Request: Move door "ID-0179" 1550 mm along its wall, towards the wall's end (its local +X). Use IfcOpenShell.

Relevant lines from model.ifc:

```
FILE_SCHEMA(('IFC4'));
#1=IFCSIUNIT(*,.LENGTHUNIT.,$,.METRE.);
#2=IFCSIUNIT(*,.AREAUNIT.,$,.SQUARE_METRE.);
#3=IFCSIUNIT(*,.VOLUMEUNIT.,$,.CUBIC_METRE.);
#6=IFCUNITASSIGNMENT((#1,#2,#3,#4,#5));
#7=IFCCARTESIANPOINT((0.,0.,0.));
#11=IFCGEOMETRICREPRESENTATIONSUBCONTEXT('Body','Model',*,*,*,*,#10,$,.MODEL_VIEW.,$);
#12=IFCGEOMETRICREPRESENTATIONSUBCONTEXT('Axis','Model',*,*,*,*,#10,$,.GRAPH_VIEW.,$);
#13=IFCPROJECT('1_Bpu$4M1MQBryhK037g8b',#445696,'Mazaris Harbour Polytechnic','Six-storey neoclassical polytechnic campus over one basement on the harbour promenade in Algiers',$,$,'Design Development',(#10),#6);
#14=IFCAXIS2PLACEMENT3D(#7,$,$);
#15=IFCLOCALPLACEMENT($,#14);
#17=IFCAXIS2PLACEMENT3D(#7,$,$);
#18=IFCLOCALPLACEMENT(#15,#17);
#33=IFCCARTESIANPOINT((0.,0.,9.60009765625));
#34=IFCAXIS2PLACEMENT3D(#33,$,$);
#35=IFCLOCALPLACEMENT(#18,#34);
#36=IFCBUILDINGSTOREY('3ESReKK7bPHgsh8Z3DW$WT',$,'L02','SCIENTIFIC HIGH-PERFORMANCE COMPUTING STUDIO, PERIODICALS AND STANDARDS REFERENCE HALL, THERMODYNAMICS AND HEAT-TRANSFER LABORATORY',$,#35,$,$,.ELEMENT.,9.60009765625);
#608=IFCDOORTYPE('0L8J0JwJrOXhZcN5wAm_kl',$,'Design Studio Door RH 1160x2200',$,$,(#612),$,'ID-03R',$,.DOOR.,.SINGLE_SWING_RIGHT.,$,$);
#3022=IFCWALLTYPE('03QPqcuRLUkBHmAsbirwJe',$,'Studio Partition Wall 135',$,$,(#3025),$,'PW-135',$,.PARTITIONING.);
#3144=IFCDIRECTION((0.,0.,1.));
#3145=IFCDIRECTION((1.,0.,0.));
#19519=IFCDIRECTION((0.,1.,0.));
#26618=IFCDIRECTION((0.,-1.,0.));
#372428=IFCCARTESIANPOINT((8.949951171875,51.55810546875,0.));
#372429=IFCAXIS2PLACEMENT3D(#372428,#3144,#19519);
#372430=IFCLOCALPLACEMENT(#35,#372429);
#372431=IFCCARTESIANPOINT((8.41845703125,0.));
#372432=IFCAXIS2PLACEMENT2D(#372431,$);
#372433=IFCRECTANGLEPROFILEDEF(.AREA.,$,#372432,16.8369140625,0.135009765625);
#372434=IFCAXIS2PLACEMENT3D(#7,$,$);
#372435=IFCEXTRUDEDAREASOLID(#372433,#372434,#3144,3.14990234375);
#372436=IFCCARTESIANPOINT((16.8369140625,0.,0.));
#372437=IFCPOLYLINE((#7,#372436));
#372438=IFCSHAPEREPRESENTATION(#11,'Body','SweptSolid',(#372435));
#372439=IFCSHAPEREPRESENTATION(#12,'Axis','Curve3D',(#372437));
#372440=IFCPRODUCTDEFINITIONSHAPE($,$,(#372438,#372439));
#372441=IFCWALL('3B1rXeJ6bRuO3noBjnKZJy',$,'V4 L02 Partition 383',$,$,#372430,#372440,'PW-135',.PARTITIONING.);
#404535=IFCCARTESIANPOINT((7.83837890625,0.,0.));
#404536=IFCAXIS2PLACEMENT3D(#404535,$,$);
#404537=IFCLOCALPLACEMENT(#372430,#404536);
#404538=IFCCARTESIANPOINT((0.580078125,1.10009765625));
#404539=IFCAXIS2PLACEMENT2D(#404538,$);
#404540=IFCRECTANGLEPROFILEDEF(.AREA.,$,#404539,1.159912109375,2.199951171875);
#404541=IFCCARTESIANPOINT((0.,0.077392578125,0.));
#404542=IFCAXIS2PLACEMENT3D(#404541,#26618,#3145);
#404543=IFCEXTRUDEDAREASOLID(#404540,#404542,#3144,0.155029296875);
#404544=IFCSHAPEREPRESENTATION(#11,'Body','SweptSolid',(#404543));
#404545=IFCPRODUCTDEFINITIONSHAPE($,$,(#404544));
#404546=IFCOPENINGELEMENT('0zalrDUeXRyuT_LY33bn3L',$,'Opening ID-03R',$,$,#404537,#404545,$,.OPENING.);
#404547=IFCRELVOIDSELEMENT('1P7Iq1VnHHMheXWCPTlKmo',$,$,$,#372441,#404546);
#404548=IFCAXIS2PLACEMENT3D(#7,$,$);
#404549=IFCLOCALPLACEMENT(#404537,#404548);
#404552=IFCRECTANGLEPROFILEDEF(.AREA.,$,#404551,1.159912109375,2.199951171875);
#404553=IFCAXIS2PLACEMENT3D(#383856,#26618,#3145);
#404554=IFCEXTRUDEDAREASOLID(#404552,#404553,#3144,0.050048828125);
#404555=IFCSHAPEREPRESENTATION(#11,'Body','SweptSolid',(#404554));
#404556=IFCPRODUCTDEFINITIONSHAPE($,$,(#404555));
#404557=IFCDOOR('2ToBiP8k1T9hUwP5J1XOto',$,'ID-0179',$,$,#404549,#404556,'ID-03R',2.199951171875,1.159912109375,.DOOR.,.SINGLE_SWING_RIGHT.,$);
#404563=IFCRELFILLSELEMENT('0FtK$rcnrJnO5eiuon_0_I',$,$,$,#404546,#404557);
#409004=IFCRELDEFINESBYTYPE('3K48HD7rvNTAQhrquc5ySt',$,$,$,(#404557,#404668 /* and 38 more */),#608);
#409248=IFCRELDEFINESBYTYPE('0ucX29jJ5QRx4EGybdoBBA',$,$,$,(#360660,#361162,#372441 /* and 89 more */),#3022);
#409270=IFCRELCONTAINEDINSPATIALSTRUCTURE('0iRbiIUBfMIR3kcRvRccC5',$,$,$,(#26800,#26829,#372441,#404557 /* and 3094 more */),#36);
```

```python
import ifcopenshell
import ifcopenshell.api.geometry
import ifcopenshell.util.placement
import ifcopenshell.util.unit

model = ifcopenshell.open("model.ifc")
unit_scale = ifcopenshell.util.unit.calculate_unit_scale(model)

door = model.by_guid("2ToBiP8k1T9hUwP5J1XOto")
opening = door.FillsVoids[0].RelatingOpeningElement
wall = opening.VoidsElements[0].RelatingBuildingElement

wall_matrix = ifcopenshell.util.placement.get_local_placement(wall.ObjectPlacement)
shift = wall_matrix[:3, 0] * 1.55 / unit_scale
before = ifcopenshell.util.placement.get_local_placement(door.ObjectPlacement)[:3, 3].copy()

# The door is placed relative to its opening, so it follows when the opening moves.
matrix = ifcopenshell.util.placement.get_local_placement(opening.ObjectPlacement)
matrix[:3, 3] += shift
ifcopenshell.api.geometry.edit_object_placement(
    model, product=opening, matrix=matrix, is_si=False, should_transform_children=True
)

after = ifcopenshell.util.placement.get_local_placement(door.ObjectPlacement)[:3, 3]
print("door moved by", (after - before).round(3) + 0.0)

model.write("model_updated.ifc")
```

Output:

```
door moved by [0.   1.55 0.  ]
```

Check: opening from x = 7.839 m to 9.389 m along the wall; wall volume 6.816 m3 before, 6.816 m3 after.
